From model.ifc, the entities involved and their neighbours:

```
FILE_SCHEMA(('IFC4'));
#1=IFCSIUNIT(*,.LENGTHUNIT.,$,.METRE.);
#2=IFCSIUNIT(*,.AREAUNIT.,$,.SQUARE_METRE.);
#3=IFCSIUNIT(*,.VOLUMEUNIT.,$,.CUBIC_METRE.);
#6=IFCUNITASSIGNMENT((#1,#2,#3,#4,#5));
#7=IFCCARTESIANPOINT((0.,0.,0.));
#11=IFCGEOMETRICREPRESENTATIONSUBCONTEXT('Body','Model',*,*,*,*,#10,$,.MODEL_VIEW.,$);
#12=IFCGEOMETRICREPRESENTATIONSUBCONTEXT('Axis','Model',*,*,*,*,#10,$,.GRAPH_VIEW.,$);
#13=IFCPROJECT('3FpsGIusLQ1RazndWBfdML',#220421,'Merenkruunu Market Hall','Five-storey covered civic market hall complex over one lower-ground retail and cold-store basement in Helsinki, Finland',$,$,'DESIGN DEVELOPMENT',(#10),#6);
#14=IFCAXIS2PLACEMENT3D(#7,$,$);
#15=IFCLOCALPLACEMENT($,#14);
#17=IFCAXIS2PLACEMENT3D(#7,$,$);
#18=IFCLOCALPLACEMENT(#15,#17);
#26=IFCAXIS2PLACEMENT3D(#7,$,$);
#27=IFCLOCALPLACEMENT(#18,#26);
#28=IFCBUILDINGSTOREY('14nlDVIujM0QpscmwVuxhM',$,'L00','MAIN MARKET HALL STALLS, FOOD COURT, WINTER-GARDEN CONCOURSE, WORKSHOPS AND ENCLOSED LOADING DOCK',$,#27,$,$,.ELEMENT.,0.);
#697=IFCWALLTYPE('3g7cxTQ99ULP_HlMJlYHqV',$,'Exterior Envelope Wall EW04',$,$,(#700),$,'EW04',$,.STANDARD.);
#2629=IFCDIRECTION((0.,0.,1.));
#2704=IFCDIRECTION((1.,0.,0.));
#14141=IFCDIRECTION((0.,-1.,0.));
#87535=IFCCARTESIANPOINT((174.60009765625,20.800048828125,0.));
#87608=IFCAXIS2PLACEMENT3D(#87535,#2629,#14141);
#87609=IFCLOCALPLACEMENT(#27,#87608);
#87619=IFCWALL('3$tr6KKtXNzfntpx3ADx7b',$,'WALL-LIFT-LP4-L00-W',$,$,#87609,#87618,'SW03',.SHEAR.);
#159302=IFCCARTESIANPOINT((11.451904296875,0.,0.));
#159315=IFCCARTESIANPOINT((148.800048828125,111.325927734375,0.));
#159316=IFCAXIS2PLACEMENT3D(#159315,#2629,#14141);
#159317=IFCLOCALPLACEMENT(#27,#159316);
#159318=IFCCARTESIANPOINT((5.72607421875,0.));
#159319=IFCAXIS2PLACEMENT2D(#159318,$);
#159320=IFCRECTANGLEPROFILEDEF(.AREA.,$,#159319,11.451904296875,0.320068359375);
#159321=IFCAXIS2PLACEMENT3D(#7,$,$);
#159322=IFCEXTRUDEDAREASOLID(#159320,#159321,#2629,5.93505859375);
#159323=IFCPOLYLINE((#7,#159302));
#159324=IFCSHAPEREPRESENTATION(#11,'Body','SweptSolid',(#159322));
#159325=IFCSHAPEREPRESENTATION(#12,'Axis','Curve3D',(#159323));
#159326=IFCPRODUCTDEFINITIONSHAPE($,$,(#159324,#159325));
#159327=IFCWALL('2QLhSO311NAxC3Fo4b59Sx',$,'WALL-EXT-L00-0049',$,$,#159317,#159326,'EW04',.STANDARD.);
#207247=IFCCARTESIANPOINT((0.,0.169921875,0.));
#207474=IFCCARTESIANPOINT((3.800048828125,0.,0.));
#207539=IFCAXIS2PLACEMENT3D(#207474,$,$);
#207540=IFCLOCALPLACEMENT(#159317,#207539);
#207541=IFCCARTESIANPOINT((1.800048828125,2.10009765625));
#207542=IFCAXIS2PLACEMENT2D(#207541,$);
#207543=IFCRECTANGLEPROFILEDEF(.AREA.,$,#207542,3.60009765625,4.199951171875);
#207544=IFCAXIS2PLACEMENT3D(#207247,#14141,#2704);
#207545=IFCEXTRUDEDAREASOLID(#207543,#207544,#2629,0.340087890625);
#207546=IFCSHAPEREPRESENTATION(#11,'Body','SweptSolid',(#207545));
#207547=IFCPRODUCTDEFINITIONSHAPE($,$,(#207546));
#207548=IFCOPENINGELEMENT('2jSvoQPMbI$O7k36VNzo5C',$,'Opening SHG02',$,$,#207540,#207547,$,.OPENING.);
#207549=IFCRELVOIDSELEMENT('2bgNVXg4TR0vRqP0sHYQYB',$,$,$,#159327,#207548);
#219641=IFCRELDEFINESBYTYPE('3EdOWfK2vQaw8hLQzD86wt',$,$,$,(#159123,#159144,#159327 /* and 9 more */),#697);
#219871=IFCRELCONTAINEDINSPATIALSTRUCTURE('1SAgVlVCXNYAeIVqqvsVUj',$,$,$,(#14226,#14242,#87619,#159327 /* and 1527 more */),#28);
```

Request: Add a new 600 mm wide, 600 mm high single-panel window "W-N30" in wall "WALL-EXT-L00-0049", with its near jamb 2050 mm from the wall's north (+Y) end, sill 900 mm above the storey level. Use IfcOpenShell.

```python
import numpy as np
import ifcopenshell
import ifcopenshell.api.feature
import ifcopenshell.api.geometry
import ifcopenshell.api.root
import ifcopenshell.api.spatial
import ifcopenshell.geom
import ifcopenshell.util.element
import ifcopenshell.util.placement
import ifcopenshell.util.representation
import ifcopenshell.util.shape
import ifcopenshell.util.unit

model = ifcopenshell.open("model.ifc")
unit_scale = ifcopenshell.util.unit.calculate_unit_scale(model)
settings = ifcopenshell.geom.settings()


def volume(element):
    """Net volume in cubic metres, openings subtracted."""
    shape = ifcopenshell.geom.create_shape(settings, element)
    return ifcopenshell.util.shape.get_volume(shape.geometry)


wall = model.by_guid("2QLhSO311NAxC3Fo4b59Sx")
storey = ifcopenshell.util.element.get_container(wall, ifc_class="IfcBuildingStorey")
context = ifcopenshell.util.representation.get_context(model, "Model", "Body", "MODEL_VIEW")
before = volume(wall)

width, height, from_end, sill = 0.6, 0.6, 2.05, 0.9  # metres

# The wall runs along its own X axis, and the end named is its -X end.
wall_shape = ifcopenshell.geom.create_shape(settings, wall)
x, y, z = ifcopenshell.util.shape.get_vertices(wall_shape.geometry).T
start = x.min() + from_end
face, thickness = float(y.min()), float(y.max() - y.min())
wall_matrix = ifcopenshell.util.placement.get_local_placement(wall.ObjectPlacement)
level = ifcopenshell.util.placement.get_local_placement(storey.ObjectPlacement)[2, 3]


def in_wall(x, y):
    """Placement at x, y metres in the wall's axes, at sill height."""
    matrix = wall_matrix.copy()
    matrix[:, 3] = wall_matrix @ np.array([x / unit_scale, y / unit_scale, 0.0, 1.0])
    matrix[2, 3] = level + sill / unit_scale
    return matrix


# Opening: a box that overshoots both wall faces by 50 mm.
opening = ifcopenshell.api.root.create_entity(model, ifc_class="IfcOpeningElement", predefined_type="OPENING")
box = ifcopenshell.api.geometry.add_wall_representation(
    model, context=context, length=width, height=height, thickness=thickness + 0.1
)
ifcopenshell.api.geometry.assign_representation(model, product=opening, representation=box)
ifcopenshell.api.geometry.edit_object_placement(model, product=opening, matrix=in_wall(start, face - 0.05), is_si=False)
ifcopenshell.api.feature.add_feature(model, feature=opening, element=wall)

window = ifcopenshell.api.root.create_entity(model, ifc_class="IfcWindow", name="W-N30", predefined_type="WINDOW")
window.OverallWidth, window.OverallHeight = width / unit_scale, height / unit_scale
window.PartitioningType = "SINGLE_PANEL"
body = ifcopenshell.api.geometry.add_window_representation(
    model,
    context=context,
    overall_width=window.OverallWidth,
    overall_height=window.OverallHeight,
    partition_type="SINGLE_PANEL",
)
ifcopenshell.api.geometry.assign_representation(model, product=window, representation=body)
ifcopenshell.api.spatial.assign_container(model, products=[window], relating_structure=storey)
ifcopenshell.api.feature.add_filling(model, opening=opening, element=window)

# Centre the window in the wall's thickness.
ifcopenshell.api.geometry.edit_object_placement(model, product=window, matrix=in_wall(start, face), is_si=False)
window_shape = ifcopenshell.geom.create_shape(settings, window)
depth = ifcopenshell.util.shape.get_vertices(window_shape.geometry)[:, 1]
offset = face + thickness / 2 - (depth.min() + depth.max()) / 2
ifcopenshell.api.geometry.edit_object_placement(model, product=window, matrix=in_wall(start, offset), is_si=False)

after = volume(wall)

print(f"wall volume {before:.3f} -> {after:.3f} m3")

model.write("model_v2.ifc")
```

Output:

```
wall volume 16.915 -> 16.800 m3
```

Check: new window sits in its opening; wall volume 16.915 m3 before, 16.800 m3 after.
